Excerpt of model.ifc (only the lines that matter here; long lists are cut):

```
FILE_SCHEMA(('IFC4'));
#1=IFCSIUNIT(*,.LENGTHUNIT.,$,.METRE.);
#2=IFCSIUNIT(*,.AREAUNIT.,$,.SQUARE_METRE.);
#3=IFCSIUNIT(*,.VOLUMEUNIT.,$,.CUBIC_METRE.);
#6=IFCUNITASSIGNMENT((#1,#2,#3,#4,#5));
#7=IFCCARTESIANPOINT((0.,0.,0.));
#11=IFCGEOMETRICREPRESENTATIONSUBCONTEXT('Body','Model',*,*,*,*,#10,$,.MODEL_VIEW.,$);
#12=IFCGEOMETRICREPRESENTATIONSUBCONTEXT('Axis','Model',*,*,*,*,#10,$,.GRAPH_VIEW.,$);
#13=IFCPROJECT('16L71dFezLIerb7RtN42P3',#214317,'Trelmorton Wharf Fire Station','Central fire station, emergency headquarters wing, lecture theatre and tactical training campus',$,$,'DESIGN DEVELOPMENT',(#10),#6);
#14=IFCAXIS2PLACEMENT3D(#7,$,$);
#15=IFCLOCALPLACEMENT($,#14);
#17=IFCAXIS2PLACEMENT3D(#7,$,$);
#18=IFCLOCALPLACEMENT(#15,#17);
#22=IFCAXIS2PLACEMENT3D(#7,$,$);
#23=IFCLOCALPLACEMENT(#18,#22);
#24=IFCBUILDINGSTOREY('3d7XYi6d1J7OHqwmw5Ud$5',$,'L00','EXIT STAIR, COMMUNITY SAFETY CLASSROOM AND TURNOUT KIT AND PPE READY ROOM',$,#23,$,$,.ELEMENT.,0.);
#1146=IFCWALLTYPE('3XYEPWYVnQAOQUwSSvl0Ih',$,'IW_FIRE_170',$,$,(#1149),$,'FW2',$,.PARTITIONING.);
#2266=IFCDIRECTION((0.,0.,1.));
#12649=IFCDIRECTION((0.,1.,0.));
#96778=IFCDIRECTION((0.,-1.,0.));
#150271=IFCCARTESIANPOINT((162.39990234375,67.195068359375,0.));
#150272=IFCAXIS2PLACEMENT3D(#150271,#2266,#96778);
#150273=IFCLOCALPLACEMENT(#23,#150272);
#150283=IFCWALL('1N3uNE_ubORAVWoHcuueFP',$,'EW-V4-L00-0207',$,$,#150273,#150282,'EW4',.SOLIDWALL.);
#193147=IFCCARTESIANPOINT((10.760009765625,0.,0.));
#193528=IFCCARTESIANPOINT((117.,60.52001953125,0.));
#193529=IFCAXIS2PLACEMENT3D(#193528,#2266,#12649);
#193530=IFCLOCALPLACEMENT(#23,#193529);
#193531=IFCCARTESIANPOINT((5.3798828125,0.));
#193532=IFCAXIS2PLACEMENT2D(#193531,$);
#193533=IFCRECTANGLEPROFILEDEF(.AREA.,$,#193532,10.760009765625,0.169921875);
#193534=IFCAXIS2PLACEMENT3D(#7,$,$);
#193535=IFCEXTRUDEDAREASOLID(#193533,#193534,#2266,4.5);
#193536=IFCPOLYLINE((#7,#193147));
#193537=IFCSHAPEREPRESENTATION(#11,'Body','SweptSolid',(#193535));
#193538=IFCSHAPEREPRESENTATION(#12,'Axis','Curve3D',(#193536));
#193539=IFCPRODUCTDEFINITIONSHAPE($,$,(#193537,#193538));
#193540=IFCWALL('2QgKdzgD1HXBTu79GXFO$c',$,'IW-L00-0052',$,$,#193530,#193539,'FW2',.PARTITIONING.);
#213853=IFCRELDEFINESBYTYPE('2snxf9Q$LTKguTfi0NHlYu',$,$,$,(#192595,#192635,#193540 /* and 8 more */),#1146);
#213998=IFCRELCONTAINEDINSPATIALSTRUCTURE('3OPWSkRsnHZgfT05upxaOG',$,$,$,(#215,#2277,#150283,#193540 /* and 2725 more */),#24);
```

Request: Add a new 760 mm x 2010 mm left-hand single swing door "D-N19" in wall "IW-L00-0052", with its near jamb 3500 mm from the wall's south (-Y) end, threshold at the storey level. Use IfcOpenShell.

```python
import numpy as np
import ifcopenshell
import ifcopenshell.api.feature
import ifcopenshell.api.geometry
import ifcopenshell.api.root
import ifcopenshell.api.spatial
import ifcopenshell.geom
import ifcopenshell.util.element
import ifcopenshell.util.placement
import ifcopenshell.util.representation
import ifcopenshell.util.shape
import ifcopenshell.util.unit

model = ifcopenshell.open("model.ifc")
unit_scale = ifcopenshell.util.unit.calculate_unit_scale(model)
settings = ifcopenshell.geom.settings()


def volume(element):
    """Net volume in cubic metres, openings subtracted."""
    shape = ifcopenshell.geom.create_shape(settings, element)
    return ifcopenshell.util.shape.get_volume(shape.geometry)


wall = model.by_id(193540)
storey = ifcopenshell.util.element.get_container(wall, ifc_class="IfcBuildingStorey")
context = ifcopenshell.util.representation.get_context(model, "Model", "Body", "MODEL_VIEW")
before = volume(wall)

width, height, from_end, sill = 0.76, 2.01, 3.5, 0.0  # metres

# The wall runs along its own X axis, and the end named is its -X end.
wall_shape = ifcopenshell.geom.create_shape(settings, wall)
x, y, z = ifcopenshell.util.shape.get_vertices(wall_shape.geometry).T
start = x.min() + from_end
face, thickness = float(y.min()), float(y.max() - y.min())
wall_matrix = ifcopenshell.util.placement.get_local_placement(wall.ObjectPlacement)
level = ifcopenshell.util.placement.get_local_placement(storey.ObjectPlacement)[2, 3]


def in_wall(x, y):
    """Placement at x, y metres in the wall's axes, at sill height."""
    matrix = wall_matrix.copy()
    matrix[:, 3] = wall_matrix @ np.array([x / unit_scale, y / unit_scale, 0.0, 1.0])
    matrix[2, 3] = level + sill / unit_scale
    return matrix


# Opening: a box that overshoots both wall faces by 50 mm.
opening = ifcopenshell.api.root.create_entity(model, ifc_class="IfcOpeningElement", predefined_type="OPENING")
box = ifcopenshell.api.geometry.add_wall_representation(
    model, context=context, length=width, height=height, thickness=thickness + 0.1
)
ifcopenshell.api.geometry.assign_representation(model, product=opening, representation=box)
ifcopenshell.api.geometry.edit_object_placement(model, product=opening, matrix=in_wall(start, face - 0.05), is_si=False)
ifcopenshell.api.feature.add_feature(model, feature=opening, element=wall)

door = ifcopenshell.api.root.create_entity(model, ifc_class="IfcDoor", name="D-N19", predefined_type="DOOR")
door.OverallWidth, door.OverallHeight = width / unit_scale, height / unit_scale
door.OperationType = "SINGLE_SWING_LEFT"
body = ifcopenshell.api.geometry.add_door_representation(
    model,
    context=context,
    overall_width=door.OverallWidth,
    overall_height=door.OverallHeight,
    operation_type="SINGLE_SWING_LEFT",
    lining_properties={"LiningDepth": thickness / unit_scale, "ThresholdDepth": thickness / unit_scale},
)
ifcopenshell.api.geometry.assign_representation(model, product=door, representation=body)
ifcopenshell.api.spatial.assign_container(model, products=[door], relating_structure=storey)
ifcopenshell.api.feature.add_filling(model, opening=opening, element=door)

# The lining spans the wall, so the door starts at the wall face.
ifcopenshell.api.geometry.edit_object_placement(model, product=door, matrix=in_wall(start, face), is_si=False)

after = volume(wall)

print(f"wall volume {before:.3f} -> {after:.3f} m3")

model.write("model_v2.ifc")
```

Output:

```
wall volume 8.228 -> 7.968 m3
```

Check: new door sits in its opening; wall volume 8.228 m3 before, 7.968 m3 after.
